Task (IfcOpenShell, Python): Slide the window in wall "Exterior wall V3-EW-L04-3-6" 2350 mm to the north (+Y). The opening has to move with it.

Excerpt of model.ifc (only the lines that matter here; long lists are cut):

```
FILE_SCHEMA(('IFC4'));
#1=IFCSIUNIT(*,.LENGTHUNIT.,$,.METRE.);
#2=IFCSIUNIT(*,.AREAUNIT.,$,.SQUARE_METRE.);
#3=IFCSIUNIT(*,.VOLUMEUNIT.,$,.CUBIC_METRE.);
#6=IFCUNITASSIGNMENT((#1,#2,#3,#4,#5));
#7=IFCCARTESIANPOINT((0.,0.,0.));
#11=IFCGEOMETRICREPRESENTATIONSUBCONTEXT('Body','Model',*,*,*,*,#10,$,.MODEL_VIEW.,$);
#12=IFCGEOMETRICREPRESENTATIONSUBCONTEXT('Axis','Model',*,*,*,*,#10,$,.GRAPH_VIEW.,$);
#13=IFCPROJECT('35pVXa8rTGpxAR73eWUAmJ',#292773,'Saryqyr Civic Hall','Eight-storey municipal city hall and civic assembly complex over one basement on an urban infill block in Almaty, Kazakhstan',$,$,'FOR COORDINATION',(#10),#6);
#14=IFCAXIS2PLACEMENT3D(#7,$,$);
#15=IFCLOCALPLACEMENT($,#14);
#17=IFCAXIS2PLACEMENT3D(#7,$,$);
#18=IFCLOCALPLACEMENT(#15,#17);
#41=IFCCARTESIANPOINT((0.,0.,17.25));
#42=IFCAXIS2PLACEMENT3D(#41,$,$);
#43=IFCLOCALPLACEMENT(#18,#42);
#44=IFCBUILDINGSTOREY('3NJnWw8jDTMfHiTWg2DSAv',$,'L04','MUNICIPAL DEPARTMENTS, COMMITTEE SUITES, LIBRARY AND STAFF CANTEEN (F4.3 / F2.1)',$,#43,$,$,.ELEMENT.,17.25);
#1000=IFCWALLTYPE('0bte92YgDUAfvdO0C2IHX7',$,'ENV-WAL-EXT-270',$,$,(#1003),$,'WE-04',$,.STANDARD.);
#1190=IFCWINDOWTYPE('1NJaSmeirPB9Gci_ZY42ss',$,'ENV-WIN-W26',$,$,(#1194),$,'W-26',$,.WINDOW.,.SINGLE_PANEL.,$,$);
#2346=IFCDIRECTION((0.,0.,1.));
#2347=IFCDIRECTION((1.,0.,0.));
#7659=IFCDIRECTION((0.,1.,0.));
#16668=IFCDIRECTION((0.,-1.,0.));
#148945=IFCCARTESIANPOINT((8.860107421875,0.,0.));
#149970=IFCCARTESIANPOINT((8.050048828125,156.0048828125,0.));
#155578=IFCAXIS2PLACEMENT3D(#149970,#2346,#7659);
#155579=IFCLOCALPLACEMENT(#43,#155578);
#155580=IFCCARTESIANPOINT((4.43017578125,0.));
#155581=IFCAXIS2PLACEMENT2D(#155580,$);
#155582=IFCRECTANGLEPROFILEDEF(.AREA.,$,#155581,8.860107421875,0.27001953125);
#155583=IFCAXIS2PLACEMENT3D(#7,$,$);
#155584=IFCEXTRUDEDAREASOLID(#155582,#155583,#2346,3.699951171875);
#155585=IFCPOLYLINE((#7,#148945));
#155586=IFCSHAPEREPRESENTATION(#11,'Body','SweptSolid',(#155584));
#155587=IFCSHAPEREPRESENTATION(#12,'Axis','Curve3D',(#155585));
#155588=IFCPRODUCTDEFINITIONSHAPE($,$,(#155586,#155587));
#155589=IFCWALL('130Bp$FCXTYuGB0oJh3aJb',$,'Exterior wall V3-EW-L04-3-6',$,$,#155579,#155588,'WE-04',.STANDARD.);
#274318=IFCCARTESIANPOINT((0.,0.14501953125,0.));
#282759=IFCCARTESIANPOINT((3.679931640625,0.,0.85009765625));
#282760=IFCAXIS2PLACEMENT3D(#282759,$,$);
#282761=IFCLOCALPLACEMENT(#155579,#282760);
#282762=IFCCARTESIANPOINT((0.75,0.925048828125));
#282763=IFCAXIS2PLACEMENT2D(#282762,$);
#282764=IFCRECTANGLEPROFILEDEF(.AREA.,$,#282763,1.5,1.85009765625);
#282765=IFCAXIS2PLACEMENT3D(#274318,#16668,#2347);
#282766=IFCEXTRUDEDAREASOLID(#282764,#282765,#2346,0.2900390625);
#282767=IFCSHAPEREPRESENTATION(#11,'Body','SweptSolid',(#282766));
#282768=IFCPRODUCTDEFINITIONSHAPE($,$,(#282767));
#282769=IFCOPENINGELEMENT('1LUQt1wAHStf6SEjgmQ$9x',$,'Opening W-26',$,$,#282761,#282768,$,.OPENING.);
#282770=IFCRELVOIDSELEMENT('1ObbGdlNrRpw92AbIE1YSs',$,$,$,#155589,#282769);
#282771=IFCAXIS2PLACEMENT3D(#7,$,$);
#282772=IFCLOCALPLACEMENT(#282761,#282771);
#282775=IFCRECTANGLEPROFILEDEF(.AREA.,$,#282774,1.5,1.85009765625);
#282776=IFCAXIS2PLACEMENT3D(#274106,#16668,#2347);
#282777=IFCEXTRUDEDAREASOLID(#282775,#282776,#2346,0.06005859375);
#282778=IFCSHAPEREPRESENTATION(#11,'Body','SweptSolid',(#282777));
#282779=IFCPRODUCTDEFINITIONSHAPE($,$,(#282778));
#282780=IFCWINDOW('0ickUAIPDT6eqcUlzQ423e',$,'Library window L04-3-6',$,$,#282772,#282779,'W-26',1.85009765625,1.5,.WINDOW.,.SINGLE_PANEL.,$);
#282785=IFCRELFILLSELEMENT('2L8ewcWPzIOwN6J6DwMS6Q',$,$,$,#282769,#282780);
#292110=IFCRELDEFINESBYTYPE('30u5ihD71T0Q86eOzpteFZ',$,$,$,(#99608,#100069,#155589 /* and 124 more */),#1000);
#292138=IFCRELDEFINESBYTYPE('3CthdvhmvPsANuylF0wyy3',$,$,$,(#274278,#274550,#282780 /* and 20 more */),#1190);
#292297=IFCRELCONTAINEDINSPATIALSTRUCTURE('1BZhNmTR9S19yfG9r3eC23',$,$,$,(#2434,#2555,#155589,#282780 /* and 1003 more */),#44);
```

```python
import ifcopenshell
import ifcopenshell.api.geometry
import ifcopenshell.util.placement
import ifcopenshell.util.unit

model = ifcopenshell.open("model.ifc")
unit_scale = ifcopenshell.util.unit.calculate_unit_scale(model)

window = model.by_guid("0ickUAIPDT6eqcUlzQ423e")
opening = window.FillsVoids[0].RelatingOpeningElement
wall = opening.VoidsElements[0].RelatingBuildingElement

wall_matrix = ifcopenshell.util.placement.get_local_placement(wall.ObjectPlacement)
shift = wall_matrix[:3, 0] * 2.35 / unit_scale
before = ifcopenshell.util.placement.get_local_placement(window.ObjectPlacement)[:3, 3].copy()

# The window is placed relative to its opening, so it follows when the opening moves.
matrix = ifcopenshell.util.placement.get_local_placement(opening.ObjectPlacement)
matrix[:3, 3] += shift
ifcopenshell.api.geometry.edit_object_placement(
    model, product=opening, matrix=matrix, is_si=False, should_transform_children=True
)

after = ifcopenshell.util.placement.get_local_placement(window.ObjectPlacement)[:3, 3]
print("window moved by", (after - before).round(3) + 0.0)

model.write("model_edited.ifc")
```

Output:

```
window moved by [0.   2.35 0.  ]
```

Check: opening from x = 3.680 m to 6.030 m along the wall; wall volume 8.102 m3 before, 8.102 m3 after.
